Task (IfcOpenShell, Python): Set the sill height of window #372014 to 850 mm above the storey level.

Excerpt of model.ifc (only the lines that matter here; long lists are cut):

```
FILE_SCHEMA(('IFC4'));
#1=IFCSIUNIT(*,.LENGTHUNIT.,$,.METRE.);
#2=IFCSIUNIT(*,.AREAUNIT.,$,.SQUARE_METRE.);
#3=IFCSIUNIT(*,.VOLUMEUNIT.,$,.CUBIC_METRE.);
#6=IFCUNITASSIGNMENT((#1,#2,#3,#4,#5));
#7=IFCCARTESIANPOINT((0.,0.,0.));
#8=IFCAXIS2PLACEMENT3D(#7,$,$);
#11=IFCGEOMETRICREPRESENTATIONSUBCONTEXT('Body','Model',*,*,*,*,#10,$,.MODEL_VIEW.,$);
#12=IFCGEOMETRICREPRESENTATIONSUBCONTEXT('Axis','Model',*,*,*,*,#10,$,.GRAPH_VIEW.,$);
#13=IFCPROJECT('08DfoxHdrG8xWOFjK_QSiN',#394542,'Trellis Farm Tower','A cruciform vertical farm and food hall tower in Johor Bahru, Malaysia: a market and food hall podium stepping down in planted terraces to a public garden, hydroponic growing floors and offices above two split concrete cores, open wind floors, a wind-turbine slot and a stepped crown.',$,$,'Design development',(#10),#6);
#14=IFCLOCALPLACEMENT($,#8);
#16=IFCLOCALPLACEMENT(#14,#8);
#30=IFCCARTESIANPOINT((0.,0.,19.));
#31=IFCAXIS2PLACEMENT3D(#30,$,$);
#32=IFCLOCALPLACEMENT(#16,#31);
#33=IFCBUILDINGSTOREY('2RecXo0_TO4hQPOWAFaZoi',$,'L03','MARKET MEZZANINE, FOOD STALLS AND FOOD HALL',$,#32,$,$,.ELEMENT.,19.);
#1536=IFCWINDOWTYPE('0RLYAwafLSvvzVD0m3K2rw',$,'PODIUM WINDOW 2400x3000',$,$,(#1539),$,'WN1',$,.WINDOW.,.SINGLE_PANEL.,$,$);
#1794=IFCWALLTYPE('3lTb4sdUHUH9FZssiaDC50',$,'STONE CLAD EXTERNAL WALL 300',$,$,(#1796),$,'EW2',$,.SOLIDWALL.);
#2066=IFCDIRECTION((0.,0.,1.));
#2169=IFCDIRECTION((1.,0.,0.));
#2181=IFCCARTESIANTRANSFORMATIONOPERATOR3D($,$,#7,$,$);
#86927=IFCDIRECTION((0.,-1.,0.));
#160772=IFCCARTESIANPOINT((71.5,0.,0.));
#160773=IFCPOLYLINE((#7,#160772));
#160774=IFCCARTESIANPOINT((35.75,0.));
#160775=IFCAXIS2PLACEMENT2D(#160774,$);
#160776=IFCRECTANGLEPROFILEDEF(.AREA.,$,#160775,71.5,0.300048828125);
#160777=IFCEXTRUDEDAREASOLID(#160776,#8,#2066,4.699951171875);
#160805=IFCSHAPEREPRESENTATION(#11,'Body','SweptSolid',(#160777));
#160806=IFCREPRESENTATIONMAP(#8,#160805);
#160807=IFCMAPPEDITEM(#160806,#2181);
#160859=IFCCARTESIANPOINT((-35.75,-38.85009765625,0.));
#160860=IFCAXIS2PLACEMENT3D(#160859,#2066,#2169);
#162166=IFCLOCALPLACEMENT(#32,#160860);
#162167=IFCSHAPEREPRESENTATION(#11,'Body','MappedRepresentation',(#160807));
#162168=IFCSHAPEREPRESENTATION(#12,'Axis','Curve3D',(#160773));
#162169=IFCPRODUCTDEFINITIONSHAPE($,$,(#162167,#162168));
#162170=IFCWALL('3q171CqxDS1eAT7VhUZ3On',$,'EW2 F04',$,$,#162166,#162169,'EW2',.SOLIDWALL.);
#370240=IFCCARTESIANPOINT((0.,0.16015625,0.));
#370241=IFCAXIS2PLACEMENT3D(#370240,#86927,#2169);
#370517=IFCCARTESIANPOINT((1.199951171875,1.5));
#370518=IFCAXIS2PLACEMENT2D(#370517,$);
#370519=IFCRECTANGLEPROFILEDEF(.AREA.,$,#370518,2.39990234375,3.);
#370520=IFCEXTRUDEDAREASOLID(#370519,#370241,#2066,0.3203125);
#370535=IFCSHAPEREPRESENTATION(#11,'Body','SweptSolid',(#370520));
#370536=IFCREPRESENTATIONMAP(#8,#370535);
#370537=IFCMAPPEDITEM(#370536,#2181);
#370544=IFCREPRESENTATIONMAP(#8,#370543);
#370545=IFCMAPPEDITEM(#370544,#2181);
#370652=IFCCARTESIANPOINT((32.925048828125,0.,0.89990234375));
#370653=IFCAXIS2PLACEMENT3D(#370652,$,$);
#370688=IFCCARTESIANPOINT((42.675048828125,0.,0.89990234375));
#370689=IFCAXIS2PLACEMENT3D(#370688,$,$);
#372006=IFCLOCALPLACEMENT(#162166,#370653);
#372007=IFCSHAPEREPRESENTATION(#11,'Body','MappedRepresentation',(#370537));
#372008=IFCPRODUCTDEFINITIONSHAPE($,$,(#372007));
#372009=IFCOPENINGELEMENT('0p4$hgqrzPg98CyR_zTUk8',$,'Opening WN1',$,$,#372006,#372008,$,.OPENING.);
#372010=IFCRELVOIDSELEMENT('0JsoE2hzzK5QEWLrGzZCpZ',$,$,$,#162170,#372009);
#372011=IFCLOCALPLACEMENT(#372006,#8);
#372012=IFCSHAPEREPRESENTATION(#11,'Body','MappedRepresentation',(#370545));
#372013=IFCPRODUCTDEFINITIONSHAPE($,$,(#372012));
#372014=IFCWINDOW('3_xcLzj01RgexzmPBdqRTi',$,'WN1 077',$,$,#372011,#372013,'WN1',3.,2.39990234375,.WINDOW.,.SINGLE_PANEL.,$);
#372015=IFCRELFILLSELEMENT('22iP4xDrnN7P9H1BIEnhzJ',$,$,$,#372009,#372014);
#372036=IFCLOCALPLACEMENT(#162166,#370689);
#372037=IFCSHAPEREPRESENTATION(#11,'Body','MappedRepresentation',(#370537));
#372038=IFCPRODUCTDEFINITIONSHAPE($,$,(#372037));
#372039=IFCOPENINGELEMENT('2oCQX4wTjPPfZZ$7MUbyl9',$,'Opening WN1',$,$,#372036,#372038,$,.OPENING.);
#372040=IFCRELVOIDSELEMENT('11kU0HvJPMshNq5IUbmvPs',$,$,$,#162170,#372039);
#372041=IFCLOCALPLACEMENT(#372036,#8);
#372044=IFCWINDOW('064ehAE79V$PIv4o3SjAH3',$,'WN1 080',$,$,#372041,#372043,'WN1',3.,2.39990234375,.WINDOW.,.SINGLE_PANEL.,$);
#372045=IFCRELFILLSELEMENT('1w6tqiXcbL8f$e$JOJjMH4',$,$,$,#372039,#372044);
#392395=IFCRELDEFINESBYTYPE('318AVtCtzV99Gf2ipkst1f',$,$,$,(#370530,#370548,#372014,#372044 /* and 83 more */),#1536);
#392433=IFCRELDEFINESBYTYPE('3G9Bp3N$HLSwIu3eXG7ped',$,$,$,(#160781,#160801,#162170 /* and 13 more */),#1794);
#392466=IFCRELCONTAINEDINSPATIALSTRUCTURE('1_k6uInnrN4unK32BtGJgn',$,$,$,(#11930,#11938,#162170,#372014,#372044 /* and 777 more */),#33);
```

```python
import numpy as np
import ifcopenshell
import ifcopenshell.api.geometry
import ifcopenshell.geom
import ifcopenshell.util.element
import ifcopenshell.util.placement
import ifcopenshell.util.shape
import ifcopenshell.util.unit

model = ifcopenshell.open("model.ifc")
unit_scale = ifcopenshell.util.unit.calculate_unit_scale(model)

window = model.by_guid("3_xcLzj01RgexzmPBdqRTi")
opening = window.FillsVoids[0].RelatingOpeningElement
storey = ifcopenshell.util.element.get_container(window, ifc_class="IfcBuildingStorey")
level = ifcopenshell.util.placement.get_local_placement(storey.ObjectPlacement)[2, 3]

# The opening's origin need not be at the sill, so measure its lowest point.
shape = ifcopenshell.geom.create_shape(ifcopenshell.geom.settings(), opening)
bottom = ifcopenshell.util.shape.get_shape_bottom_elevation(shape, shape.geometry) / unit_scale
dz = level + 0.85 - bottom

shift = np.array([0.0, 0.0, dz])
# The window is placed relative to its opening, so it follows when the opening moves.
matrix = ifcopenshell.util.placement.get_local_placement(opening.ObjectPlacement)
matrix[:3, 3] += shift
ifcopenshell.api.geometry.edit_object_placement(
    model, product=opening, matrix=matrix, is_si=False, should_transform_children=True
)

print(f"moved by {dz * unit_scale:+.3f} m")

model.write("model_v2.ifc")
```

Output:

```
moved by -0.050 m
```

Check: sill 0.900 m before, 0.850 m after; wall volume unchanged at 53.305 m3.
